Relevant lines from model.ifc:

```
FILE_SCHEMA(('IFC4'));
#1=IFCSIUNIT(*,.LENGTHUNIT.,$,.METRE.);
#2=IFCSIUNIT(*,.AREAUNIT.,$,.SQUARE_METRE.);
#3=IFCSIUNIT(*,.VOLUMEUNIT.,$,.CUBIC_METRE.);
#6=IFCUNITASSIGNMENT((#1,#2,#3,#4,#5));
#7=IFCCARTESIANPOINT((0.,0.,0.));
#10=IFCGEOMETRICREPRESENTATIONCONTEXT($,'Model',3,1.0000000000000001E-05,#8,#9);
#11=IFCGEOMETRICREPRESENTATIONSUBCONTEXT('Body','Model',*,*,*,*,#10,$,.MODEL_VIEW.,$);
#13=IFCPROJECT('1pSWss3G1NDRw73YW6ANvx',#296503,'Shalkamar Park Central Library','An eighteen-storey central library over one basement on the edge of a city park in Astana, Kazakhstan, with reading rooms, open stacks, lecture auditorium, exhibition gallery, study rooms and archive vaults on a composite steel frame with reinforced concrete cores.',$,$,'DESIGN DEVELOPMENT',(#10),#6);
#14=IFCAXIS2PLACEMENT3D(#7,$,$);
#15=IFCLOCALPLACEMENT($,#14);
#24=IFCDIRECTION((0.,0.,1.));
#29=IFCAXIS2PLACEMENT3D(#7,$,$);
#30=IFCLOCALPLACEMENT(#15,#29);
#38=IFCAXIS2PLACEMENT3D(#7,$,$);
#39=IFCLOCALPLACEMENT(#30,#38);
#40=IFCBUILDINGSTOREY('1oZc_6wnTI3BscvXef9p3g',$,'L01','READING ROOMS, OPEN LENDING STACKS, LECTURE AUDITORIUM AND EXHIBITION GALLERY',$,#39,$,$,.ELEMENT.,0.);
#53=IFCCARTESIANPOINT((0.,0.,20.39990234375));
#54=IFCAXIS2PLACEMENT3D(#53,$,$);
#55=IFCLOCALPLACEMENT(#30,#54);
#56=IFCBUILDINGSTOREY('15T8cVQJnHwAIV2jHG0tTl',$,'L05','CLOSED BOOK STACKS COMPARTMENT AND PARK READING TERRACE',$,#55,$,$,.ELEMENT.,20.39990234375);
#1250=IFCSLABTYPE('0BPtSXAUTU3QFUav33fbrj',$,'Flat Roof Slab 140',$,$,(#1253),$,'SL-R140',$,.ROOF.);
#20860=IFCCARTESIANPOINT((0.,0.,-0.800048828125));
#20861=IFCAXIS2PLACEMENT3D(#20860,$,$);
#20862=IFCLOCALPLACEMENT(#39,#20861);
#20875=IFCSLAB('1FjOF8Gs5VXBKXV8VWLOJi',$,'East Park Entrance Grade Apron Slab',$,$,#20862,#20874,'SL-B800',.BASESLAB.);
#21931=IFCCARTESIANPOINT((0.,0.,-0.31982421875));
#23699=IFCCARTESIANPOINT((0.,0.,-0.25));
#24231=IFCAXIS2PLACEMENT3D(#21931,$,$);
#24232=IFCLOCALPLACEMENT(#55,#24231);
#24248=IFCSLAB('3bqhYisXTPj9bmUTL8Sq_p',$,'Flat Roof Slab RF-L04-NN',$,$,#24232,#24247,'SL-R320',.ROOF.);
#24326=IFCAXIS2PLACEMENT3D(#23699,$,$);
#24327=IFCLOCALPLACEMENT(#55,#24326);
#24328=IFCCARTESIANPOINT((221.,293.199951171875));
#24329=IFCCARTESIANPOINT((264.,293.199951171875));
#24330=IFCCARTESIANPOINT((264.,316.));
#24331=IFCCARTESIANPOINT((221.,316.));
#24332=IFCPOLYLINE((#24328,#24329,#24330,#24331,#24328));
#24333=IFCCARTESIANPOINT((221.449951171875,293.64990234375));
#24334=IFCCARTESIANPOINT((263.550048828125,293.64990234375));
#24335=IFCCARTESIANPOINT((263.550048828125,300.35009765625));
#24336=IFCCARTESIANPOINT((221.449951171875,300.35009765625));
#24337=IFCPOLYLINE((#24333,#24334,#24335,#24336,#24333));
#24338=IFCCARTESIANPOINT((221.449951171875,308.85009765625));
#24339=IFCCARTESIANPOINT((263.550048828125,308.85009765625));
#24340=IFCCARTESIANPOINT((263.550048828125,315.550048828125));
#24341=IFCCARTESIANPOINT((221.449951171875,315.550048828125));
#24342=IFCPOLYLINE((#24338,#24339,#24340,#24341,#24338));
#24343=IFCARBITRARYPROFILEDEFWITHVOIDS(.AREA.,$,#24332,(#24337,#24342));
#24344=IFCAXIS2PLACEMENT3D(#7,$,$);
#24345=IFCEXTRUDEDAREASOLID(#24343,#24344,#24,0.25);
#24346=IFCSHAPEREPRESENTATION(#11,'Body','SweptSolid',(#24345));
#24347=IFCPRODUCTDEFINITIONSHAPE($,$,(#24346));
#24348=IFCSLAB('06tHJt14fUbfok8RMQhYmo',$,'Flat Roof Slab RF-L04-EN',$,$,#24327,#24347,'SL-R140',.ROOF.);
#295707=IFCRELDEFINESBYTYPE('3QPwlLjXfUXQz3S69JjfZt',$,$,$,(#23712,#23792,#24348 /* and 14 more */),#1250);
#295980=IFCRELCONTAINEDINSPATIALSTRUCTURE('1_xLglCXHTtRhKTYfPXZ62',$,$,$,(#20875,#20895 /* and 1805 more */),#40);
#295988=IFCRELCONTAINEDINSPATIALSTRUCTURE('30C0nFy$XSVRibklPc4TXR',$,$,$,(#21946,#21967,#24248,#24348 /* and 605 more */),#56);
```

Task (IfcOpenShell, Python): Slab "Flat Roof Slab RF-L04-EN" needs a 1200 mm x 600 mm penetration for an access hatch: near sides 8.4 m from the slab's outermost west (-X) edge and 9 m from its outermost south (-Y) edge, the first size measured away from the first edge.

```python
import numpy as np
import ifcopenshell
import ifcopenshell.api.feature
import ifcopenshell.api.geometry
import ifcopenshell.api.root
import ifcopenshell.geom
import ifcopenshell.util.placement
import ifcopenshell.util.representation
import ifcopenshell.util.shape
import ifcopenshell.util.unit

model = ifcopenshell.open("model.ifc")
unit_scale = ifcopenshell.util.unit.calculate_unit_scale(model)
settings = ifcopenshell.geom.settings()


def volume(element):
    """Net volume in cubic metres, openings subtracted."""
    shape = ifcopenshell.geom.create_shape(settings, element)
    return ifcopenshell.util.shape.get_volume(shape.geometry)


slab = model.by_id(24348)
before = volume(slab)

# Extent in the slab's own axes, in metres. The edges named are its -X and -Y sides.
slab_shape = ifcopenshell.geom.create_shape(settings, slab)
vertices = ifcopenshell.util.shape.get_vertices(slab_shape.geometry)
x_min, y_min, bottom = vertices.min(axis=0)
top = vertices[:, 2].max()

opening = ifcopenshell.api.root.create_entity(model, ifc_class="IfcOpeningElement", name="Access hatch opening", predefined_type="OPENING")
context = ifcopenshell.util.representation.get_context(model, "Model", "Body", "MODEL_VIEW")
width, depth = 1.2, 0.6
outline = [(0.0, 0.0), (width, 0.0), (width, depth), (0.0, depth), (0.0, 0.0)]
# Overshoot both faces by 50 mm so the cut is clean.
shape = ifcopenshell.api.geometry.add_slab_representation(
    model, context=context, depth=top - bottom + 0.1, polyline=outline
)
ifcopenshell.api.geometry.assign_representation(model, product=opening, representation=shape)

matrix = ifcopenshell.util.placement.get_local_placement(slab.ObjectPlacement)
matrix[:, 3] = matrix @ np.append(np.array([x_min + 8.4, y_min + 9, bottom - 0.05]) / unit_scale, 1.0)
ifcopenshell.api.geometry.edit_object_placement(model, product=opening, matrix=matrix, is_si=False)
ifcopenshell.api.feature.add_feature(model, feature=opening, element=slab)

after = volume(slab)

print(f"slab volume {before:.3f} -> {after:.3f} m3")

model.write("model_updated.ifc")
```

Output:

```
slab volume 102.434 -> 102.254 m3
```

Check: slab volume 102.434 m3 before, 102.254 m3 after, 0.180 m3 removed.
